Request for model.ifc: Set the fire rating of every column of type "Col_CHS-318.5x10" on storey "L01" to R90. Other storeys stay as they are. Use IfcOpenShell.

First a look at what the model holds.

```python
import ifcopenshell
import ifcopenshell.util.element

model = ifcopenshell.open("model.ifc")
print(model.schema)
storey = next(s for s in model.by_type("IfcBuildingStorey") if s.Name == "L01")
columns = [e for e in ifcopenshell.util.element.get_decomposition(storey) if e.is_a("IfcColumn")]
seen = {}
for e in columns:
    element_type = ifcopenshell.util.element.get_type(e)
    key = (element_type.Name if element_type != e and element_type else None, ifcopenshell.util.element.get_pset(e, "Pset_ColumnCommon", "FireRating"))
    seen[key] = seen.get(key, 0) + 1
for (name, value), count in sorted(seen.items(), key=str):
    print(count, "x", name, "|", value)
```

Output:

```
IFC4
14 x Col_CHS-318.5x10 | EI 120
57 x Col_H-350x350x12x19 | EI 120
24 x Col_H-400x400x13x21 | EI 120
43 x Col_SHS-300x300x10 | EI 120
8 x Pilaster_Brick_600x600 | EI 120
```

```python
import ifcopenshell
import ifcopenshell.api.pset
import ifcopenshell.util.element

model = ifcopenshell.open("model.ifc")

storey = next(s for s in model.by_type("IfcBuildingStorey") if s.Name == "L01")
columns = [e for e in ifcopenshell.util.element.get_decomposition(storey) if e.is_a("IfcColumn")]

count = 0
for e in columns:
    element_type = ifcopenshell.util.element.get_type(e)
    if element_type in (None, e) or element_type.Name != "Col_CHS-318.5x10":
        continue
    # add_pset returns the element's existing set when there is one.
    pset = ifcopenshell.api.pset.add_pset(model, product=e, name="Pset_ColumnCommon")
    ifcopenshell.api.pset.edit_pset(model, pset=pset, properties={"FireRating": "R90"})
    count += 1

print(count, "columns updated")

model.write("model_edited.ifc")
```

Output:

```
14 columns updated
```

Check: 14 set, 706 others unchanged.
